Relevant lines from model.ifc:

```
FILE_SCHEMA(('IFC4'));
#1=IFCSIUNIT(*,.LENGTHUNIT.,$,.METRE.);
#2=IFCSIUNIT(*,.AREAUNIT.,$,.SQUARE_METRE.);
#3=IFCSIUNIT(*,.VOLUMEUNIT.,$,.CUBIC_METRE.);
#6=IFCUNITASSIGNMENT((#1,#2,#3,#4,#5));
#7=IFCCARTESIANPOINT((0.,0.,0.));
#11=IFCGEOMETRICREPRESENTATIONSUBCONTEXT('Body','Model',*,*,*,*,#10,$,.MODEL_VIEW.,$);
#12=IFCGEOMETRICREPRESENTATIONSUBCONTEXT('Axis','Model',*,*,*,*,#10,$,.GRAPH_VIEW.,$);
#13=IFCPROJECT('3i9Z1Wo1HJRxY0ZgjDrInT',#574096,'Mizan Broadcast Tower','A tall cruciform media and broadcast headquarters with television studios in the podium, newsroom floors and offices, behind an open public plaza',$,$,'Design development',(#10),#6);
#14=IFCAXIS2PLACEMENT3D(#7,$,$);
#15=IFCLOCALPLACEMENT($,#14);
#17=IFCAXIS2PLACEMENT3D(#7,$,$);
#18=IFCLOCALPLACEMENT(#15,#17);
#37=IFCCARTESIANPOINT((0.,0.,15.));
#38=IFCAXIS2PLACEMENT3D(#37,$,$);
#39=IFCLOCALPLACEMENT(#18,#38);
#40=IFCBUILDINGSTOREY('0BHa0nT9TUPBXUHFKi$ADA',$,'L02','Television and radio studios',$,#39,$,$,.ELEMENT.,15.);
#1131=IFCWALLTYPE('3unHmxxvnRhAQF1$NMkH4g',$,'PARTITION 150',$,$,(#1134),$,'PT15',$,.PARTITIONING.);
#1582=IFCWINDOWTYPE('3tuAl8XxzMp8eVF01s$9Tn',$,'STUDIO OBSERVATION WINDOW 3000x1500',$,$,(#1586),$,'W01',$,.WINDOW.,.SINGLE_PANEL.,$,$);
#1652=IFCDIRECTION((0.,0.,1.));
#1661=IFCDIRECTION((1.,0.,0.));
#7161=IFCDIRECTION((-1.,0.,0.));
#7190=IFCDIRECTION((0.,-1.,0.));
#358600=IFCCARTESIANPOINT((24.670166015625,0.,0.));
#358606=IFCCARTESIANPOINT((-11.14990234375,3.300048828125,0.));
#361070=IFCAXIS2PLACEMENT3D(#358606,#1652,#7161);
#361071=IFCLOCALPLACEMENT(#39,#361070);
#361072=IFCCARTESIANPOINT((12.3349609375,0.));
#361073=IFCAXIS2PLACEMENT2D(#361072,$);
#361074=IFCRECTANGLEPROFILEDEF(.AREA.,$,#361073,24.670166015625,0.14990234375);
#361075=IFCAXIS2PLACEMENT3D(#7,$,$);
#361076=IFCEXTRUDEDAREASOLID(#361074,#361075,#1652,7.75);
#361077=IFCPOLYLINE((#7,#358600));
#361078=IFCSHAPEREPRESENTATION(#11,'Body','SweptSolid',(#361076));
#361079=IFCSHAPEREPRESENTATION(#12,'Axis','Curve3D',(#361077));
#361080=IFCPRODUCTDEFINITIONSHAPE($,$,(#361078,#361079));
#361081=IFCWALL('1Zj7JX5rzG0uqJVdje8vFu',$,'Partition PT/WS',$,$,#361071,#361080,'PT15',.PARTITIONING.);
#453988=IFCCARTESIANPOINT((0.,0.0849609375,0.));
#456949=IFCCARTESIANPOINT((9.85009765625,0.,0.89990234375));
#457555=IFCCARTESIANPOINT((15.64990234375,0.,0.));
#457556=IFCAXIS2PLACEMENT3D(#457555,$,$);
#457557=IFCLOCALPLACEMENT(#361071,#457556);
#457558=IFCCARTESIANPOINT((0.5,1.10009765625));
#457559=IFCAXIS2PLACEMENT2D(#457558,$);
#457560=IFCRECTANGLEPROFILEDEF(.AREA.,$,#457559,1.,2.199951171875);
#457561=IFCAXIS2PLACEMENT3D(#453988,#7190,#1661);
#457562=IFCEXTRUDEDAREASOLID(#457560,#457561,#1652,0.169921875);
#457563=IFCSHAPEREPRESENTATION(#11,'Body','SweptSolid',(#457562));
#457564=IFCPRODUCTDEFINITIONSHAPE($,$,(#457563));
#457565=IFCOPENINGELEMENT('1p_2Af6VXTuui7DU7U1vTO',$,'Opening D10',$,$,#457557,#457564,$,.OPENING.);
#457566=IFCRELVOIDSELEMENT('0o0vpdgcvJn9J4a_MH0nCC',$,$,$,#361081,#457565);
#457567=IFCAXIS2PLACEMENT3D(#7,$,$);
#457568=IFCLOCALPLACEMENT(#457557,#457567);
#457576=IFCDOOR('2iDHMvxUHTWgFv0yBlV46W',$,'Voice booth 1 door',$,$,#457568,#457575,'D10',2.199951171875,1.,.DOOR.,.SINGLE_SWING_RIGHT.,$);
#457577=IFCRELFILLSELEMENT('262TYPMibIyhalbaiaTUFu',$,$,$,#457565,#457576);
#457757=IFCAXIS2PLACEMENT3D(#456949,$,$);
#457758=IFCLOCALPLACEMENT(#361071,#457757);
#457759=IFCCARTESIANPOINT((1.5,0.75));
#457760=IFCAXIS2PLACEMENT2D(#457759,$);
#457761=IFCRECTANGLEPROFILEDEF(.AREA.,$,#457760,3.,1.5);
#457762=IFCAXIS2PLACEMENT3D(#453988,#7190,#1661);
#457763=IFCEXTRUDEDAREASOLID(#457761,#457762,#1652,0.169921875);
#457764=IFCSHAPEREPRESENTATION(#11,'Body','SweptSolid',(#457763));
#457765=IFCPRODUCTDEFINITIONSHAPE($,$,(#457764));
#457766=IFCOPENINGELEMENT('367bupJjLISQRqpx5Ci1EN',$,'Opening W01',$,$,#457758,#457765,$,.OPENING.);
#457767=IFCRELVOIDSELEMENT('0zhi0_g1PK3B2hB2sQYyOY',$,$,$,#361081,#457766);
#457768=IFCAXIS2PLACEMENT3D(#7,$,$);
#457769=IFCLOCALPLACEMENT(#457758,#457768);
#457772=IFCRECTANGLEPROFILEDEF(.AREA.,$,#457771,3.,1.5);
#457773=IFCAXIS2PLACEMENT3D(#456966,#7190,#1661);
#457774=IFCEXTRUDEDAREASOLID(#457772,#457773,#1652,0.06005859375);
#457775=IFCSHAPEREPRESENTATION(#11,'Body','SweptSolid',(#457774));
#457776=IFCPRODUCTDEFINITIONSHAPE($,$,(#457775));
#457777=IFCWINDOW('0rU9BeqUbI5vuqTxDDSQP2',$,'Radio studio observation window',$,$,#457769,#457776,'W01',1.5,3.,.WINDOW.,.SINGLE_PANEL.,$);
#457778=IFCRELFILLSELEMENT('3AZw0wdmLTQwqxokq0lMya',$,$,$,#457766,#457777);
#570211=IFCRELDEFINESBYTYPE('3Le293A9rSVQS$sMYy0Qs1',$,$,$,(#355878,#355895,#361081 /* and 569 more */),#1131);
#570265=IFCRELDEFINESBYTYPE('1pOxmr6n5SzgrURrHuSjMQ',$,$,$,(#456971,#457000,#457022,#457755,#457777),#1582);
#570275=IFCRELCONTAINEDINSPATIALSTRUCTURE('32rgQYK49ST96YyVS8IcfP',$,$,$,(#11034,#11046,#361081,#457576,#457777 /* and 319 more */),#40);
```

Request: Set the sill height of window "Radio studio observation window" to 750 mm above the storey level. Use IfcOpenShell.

```python
import numpy as np
import ifcopenshell
import ifcopenshell.api.geometry
import ifcopenshell.geom
import ifcopenshell.util.element
import ifcopenshell.util.placement
import ifcopenshell.util.shape
import ifcopenshell.util.unit

model = ifcopenshell.open("model.ifc")
unit_scale = ifcopenshell.util.unit.calculate_unit_scale(model)

window = model.by_guid("0rU9BeqUbI5vuqTxDDSQP2")
opening = window.FillsVoids[0].RelatingOpeningElement
storey = ifcopenshell.util.element.get_container(window, ifc_class="IfcBuildingStorey")
level = ifcopenshell.util.placement.get_local_placement(storey.ObjectPlacement)[2, 3]

# The opening's origin need not be at the sill, so measure its lowest point.
shape = ifcopenshell.geom.create_shape(ifcopenshell.geom.settings(), opening)
bottom = ifcopenshell.util.shape.get_shape_bottom_elevation(shape, shape.geometry) / unit_scale
dz = level + 0.75 / unit_scale - bottom

shift = np.array([0.0, 0.0, dz])
# The window is placed relative to its opening, so it follows when the opening moves.
matrix = ifcopenshell.util.placement.get_local_placement(opening.ObjectPlacement)
matrix[:3, 3] += shift
ifcopenshell.api.geometry.edit_object_placement(
    model, product=opening, matrix=matrix, is_si=False, should_transform_children=True
)

print(f"moved by {dz * unit_scale:+.3f} m")

model.write("model_rev.ifc")
```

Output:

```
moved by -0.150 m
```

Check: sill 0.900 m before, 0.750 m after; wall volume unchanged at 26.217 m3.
